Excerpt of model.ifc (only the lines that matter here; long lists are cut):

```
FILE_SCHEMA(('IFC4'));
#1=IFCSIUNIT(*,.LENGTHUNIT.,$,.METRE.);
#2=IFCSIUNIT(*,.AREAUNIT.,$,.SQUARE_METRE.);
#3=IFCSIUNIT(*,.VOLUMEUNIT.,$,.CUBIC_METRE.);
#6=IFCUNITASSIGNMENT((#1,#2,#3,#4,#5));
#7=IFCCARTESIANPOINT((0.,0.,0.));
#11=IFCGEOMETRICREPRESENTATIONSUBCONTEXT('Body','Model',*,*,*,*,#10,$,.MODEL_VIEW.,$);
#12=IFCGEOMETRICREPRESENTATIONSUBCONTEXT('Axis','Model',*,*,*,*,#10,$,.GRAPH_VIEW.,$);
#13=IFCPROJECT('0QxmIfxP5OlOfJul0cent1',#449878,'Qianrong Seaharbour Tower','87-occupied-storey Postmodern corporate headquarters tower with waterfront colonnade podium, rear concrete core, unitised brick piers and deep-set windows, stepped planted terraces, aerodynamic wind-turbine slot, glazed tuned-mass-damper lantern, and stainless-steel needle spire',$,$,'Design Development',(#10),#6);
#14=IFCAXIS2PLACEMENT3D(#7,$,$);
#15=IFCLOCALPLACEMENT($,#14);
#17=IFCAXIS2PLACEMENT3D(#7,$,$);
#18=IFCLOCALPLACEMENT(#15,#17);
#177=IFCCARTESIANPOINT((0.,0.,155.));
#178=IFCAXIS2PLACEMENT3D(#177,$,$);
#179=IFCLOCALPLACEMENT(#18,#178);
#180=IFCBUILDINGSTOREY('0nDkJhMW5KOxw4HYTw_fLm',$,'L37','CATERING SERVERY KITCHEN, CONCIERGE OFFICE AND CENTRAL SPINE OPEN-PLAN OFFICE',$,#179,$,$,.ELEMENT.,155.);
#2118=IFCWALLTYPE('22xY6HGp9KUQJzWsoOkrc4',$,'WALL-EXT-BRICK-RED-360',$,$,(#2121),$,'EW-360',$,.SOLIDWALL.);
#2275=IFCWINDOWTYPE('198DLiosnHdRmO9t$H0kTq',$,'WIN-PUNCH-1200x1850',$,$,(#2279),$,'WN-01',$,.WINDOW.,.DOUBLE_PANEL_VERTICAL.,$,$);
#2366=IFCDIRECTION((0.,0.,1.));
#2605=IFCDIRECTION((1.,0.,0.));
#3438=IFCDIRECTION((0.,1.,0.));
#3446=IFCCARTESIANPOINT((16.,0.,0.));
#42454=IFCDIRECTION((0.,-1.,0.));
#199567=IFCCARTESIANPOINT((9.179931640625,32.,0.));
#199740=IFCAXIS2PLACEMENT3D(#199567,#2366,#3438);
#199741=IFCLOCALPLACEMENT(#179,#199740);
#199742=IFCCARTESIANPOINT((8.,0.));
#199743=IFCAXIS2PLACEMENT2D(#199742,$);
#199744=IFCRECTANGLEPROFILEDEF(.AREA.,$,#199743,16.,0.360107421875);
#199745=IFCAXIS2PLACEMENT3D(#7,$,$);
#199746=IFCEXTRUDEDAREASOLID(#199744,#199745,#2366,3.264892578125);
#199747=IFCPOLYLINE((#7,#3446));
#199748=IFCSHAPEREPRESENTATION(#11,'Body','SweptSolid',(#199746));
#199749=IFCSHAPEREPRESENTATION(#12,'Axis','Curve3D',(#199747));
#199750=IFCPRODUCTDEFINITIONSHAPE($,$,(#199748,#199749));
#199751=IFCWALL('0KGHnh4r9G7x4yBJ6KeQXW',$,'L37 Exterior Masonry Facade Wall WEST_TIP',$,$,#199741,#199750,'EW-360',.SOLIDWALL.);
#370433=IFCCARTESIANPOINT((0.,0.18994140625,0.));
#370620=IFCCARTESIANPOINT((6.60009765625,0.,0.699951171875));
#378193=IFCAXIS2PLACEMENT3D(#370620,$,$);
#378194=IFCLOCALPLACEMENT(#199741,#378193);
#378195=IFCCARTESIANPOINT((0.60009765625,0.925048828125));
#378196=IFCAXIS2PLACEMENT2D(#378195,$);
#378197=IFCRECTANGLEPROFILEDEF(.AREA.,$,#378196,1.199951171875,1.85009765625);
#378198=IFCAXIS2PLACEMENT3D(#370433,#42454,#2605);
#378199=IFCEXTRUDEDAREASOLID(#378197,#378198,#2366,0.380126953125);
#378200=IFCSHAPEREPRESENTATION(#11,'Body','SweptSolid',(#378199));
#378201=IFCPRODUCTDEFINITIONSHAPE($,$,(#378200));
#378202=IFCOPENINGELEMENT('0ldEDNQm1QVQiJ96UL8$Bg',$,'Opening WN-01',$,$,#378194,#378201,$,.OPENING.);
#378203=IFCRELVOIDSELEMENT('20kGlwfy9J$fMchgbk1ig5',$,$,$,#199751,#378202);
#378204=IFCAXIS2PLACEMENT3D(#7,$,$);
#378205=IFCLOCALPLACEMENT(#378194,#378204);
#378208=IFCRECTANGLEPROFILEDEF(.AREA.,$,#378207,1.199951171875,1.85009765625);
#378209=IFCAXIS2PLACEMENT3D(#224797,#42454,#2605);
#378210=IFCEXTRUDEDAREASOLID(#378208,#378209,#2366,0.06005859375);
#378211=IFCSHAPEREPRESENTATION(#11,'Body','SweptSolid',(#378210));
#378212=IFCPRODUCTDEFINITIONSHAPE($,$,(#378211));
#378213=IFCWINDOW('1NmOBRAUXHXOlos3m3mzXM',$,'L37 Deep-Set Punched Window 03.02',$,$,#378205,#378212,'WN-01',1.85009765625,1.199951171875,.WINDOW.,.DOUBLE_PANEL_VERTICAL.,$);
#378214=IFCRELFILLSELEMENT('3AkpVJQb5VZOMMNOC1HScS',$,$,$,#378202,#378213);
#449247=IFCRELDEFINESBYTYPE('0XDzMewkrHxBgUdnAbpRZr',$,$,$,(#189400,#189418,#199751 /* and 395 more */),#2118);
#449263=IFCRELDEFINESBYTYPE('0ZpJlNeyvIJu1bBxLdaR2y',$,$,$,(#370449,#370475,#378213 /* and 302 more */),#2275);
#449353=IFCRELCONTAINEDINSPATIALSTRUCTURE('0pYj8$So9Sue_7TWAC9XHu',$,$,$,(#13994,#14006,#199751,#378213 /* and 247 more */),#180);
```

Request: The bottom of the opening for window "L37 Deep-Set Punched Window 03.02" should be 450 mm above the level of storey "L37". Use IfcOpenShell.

```python
import numpy as np
import ifcopenshell
import ifcopenshell.api.geometry
import ifcopenshell.geom
import ifcopenshell.util.element
import ifcopenshell.util.placement
import ifcopenshell.util.shape
import ifcopenshell.util.unit

model = ifcopenshell.open("model.ifc")
unit_scale = ifcopenshell.util.unit.calculate_unit_scale(model)

window = model.by_guid("1NmOBRAUXHXOlos3m3mzXM")
opening = window.FillsVoids[0].RelatingOpeningElement
storey = ifcopenshell.util.element.get_container(window, ifc_class="IfcBuildingStorey")
level = ifcopenshell.util.placement.get_local_placement(storey.ObjectPlacement)[2, 3]

# The opening's origin need not be at the sill, so measure its lowest point.
shape = ifcopenshell.geom.create_shape(ifcopenshell.geom.settings(), opening)
bottom = ifcopenshell.util.shape.get_shape_bottom_elevation(shape, shape.geometry) / unit_scale
dz = level + 0.45 - bottom

shift = np.array([0.0, 0.0, dz])
# The window is placed relative to its opening, so it follows when the opening moves.
matrix = ifcopenshell.util.placement.get_local_placement(opening.ObjectPlacement)
matrix[:3, 3] += shift
ifcopenshell.api.geometry.edit_object_placement(
    model, product=opening, matrix=matrix, is_si=False, should_transform_children=True
)

print(f"moved by {dz * unit_scale:+.3f} m")

model.write("model_updated.ifc")
```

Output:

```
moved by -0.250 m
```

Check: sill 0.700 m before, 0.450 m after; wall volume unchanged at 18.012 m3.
